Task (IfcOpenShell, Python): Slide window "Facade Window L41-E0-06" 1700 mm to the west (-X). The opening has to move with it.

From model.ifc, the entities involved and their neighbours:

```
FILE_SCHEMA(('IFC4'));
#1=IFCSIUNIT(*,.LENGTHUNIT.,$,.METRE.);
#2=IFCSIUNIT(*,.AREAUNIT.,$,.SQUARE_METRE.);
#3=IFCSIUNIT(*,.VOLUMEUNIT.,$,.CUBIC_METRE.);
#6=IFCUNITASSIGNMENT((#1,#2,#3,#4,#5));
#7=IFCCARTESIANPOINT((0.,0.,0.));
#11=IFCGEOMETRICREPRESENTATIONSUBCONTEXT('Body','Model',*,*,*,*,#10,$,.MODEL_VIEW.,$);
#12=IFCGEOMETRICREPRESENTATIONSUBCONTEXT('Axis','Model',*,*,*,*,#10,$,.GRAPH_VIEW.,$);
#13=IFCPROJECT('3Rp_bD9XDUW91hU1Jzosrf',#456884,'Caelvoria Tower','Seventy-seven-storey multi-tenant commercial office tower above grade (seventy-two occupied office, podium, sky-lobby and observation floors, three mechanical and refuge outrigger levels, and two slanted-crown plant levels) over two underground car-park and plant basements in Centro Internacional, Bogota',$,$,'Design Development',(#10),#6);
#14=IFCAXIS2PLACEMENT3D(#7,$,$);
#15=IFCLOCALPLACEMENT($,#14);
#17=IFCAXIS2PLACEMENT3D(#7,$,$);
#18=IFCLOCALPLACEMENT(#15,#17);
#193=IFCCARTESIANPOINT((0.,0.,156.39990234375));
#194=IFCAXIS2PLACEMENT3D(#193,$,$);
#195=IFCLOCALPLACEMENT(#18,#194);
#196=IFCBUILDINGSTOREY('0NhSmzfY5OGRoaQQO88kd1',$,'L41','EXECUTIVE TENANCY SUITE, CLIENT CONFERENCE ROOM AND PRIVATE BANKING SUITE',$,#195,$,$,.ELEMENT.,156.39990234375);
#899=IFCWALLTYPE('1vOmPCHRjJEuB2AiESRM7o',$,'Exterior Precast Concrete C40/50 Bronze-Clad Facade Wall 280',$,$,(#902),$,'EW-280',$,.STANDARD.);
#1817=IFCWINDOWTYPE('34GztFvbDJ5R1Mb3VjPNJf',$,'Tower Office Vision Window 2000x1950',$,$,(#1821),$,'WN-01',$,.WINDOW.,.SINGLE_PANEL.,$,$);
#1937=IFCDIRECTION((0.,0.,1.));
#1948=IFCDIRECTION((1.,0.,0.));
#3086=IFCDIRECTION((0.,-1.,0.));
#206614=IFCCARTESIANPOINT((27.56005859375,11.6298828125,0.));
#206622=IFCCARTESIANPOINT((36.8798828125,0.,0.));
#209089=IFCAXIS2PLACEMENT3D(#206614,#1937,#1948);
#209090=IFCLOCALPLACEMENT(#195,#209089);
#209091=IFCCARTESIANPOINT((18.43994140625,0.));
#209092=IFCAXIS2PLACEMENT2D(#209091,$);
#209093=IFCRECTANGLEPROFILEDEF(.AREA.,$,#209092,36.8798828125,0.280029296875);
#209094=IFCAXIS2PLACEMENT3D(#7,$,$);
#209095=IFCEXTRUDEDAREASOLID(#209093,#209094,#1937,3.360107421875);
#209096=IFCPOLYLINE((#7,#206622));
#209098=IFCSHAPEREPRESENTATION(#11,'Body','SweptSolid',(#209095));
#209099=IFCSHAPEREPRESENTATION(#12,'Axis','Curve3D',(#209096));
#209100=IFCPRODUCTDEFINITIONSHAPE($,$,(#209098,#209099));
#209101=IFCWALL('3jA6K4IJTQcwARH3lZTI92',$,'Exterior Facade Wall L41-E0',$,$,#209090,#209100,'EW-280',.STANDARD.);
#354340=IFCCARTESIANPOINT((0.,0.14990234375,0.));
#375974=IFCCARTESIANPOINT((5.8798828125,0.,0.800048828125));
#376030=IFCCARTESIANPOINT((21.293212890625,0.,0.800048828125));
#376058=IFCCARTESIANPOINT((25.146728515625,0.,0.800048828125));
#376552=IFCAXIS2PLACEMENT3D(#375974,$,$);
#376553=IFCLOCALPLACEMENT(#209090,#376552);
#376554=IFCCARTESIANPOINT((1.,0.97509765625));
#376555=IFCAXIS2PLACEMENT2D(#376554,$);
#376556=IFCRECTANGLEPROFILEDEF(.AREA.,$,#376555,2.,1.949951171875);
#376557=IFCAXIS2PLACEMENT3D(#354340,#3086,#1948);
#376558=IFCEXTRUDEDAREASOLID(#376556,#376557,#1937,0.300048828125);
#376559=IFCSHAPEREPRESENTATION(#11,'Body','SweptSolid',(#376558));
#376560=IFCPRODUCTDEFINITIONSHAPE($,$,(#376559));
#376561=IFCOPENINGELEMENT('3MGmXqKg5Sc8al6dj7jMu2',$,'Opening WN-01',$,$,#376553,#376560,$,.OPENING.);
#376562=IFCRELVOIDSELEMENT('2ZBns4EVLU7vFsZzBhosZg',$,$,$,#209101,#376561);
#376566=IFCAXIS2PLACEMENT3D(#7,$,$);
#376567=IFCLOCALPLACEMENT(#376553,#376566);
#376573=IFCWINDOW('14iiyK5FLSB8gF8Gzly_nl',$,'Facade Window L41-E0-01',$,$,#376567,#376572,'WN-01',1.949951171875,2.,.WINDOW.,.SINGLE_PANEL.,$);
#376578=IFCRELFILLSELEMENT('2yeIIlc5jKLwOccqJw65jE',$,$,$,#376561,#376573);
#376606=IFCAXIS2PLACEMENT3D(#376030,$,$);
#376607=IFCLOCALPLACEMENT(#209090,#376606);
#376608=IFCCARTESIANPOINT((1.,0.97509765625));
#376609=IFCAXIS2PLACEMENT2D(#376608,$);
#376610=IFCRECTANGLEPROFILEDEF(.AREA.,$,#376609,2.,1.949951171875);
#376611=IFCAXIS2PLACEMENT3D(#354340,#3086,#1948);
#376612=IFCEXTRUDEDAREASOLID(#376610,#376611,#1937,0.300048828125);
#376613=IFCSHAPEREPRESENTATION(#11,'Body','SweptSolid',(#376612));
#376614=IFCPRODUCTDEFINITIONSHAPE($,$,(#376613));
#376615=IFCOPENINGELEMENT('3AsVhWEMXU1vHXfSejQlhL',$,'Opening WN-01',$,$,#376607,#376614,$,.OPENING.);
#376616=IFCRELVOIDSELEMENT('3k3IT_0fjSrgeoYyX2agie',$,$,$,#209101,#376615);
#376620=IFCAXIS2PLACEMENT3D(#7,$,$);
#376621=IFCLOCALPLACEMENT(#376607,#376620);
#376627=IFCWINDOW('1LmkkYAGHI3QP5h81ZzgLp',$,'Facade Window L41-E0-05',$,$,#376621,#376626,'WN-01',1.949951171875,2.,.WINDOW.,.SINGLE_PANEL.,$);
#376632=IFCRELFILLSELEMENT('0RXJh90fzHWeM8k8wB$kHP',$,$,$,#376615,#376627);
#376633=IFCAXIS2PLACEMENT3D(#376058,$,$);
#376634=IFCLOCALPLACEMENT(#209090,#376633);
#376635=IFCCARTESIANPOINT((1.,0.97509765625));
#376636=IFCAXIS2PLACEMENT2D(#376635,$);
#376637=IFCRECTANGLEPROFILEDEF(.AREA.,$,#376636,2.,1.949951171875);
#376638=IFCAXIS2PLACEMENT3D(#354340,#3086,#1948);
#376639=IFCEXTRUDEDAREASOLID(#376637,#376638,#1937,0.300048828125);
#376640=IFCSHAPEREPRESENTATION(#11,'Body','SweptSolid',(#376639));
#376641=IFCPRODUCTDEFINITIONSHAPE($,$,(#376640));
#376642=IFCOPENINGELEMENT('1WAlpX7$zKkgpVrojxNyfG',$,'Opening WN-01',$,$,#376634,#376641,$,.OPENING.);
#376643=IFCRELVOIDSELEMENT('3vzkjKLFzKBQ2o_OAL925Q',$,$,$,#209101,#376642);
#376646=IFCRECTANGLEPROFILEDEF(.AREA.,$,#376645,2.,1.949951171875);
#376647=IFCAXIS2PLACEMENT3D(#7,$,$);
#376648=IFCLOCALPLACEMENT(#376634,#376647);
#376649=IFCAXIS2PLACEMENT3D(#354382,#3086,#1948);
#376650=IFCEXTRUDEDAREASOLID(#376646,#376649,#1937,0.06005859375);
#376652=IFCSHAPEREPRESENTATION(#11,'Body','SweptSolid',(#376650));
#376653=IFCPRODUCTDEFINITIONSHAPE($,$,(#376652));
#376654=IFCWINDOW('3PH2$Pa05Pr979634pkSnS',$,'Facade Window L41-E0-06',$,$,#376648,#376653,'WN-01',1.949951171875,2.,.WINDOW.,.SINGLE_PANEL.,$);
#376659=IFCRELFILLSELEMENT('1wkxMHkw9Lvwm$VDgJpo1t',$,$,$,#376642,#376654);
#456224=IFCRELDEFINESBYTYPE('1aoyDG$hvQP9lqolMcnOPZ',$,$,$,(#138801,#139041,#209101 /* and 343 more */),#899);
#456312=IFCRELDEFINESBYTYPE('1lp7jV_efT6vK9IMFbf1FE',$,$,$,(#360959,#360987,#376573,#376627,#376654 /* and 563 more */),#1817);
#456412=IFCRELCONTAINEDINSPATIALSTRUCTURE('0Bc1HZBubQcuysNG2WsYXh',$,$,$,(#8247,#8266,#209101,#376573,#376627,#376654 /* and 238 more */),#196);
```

```python
import ifcopenshell
import ifcopenshell.api.geometry
import ifcopenshell.util.placement
import ifcopenshell.util.unit

model = ifcopenshell.open("model.ifc")
unit_scale = ifcopenshell.util.unit.calculate_unit_scale(model)

window = model.by_guid("3PH2$Pa05Pr979634pkSnS")
opening = window.FillsVoids[0].RelatingOpeningElement
wall = opening.VoidsElements[0].RelatingBuildingElement

wall_matrix = ifcopenshell.util.placement.get_local_placement(wall.ObjectPlacement)
shift = wall_matrix[:3, 0] * -1.7 / unit_scale
before = ifcopenshell.util.placement.get_local_placement(window.ObjectPlacement)[:3, 3].copy()

# The window is placed relative to its opening, so it follows when the opening moves.
matrix = ifcopenshell.util.placement.get_local_placement(opening.ObjectPlacement)
matrix[:3, 3] += shift
ifcopenshell.api.geometry.edit_object_placement(
    model, product=opening, matrix=matrix, is_si=False, should_transform_children=True
)

after = ifcopenshell.util.placement.get_local_placement(window.ObjectPlacement)[:3, 3]
print("window moved by", (after - before).round(3) + 0.0)

model.write("model_v2.ifc")
```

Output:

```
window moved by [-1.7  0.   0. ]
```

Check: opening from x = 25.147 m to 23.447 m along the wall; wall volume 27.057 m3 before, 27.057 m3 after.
